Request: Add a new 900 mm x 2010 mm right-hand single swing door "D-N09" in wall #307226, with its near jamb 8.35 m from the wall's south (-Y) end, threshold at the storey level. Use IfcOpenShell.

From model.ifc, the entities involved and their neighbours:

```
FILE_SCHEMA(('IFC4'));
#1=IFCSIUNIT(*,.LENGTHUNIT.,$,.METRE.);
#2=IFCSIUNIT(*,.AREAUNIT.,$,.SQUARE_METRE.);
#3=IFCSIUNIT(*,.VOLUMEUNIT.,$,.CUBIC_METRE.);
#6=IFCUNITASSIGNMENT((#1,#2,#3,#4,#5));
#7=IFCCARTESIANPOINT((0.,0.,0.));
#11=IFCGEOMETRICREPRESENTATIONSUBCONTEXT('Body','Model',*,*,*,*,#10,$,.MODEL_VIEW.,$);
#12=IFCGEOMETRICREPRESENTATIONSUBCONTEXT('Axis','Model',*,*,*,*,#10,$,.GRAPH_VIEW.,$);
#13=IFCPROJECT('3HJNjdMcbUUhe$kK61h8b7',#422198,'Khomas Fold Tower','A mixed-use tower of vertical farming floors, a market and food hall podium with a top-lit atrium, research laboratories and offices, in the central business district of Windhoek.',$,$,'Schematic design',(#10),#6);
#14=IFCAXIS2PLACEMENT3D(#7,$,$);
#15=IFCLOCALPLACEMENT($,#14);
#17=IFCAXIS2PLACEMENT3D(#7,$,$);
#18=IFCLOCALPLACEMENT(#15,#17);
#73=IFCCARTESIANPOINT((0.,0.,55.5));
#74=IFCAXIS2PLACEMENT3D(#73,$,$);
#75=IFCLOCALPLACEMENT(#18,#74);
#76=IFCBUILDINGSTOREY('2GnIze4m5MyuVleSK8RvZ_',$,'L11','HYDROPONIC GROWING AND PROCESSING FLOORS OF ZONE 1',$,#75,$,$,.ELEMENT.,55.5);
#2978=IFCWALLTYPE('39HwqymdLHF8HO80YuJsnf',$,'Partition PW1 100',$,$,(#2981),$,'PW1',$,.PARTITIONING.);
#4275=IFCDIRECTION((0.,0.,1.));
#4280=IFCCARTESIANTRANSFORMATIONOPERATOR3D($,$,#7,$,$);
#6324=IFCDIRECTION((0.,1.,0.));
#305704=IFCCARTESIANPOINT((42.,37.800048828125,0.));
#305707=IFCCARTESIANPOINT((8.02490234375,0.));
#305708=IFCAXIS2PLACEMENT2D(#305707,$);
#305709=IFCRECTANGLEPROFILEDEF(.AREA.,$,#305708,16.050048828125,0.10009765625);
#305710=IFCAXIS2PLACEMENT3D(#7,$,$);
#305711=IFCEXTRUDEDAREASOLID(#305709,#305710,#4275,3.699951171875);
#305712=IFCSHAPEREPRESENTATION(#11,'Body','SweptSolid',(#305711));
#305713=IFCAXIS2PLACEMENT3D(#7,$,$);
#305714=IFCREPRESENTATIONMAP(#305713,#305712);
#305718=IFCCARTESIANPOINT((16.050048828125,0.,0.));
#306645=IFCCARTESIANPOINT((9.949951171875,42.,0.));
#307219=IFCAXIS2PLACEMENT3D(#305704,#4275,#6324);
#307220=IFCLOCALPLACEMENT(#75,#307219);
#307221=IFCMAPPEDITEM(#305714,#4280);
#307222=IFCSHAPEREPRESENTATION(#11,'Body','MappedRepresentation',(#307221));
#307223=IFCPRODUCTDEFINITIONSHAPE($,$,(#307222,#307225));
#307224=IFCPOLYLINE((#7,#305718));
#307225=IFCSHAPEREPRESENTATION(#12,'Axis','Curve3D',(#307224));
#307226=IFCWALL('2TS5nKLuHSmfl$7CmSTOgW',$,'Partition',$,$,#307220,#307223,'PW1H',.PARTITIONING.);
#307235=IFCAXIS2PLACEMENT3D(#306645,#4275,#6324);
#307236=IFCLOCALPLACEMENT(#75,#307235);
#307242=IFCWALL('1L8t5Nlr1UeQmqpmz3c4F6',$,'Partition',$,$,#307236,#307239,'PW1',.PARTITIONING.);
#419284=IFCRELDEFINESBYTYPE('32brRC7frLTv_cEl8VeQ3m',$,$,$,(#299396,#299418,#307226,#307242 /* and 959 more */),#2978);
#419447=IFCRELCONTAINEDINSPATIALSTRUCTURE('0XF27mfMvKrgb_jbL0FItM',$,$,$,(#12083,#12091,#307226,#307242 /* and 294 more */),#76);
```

```python
import numpy as np
import ifcopenshell
import ifcopenshell.api.feature
import ifcopenshell.api.geometry
import ifcopenshell.api.root
import ifcopenshell.api.spatial
import ifcopenshell.geom
import ifcopenshell.util.element
import ifcopenshell.util.placement
import ifcopenshell.util.representation
import ifcopenshell.util.shape
import ifcopenshell.util.unit

model = ifcopenshell.open("model.ifc")
unit_scale = ifcopenshell.util.unit.calculate_unit_scale(model)
settings = ifcopenshell.geom.settings()


def volume(element):
    """Net volume in cubic metres, openings subtracted."""
    shape = ifcopenshell.geom.create_shape(settings, element)
    return ifcopenshell.util.shape.get_volume(shape.geometry)


wall = model.by_guid("2TS5nKLuHSmfl$7CmSTOgW")
storey = ifcopenshell.util.element.get_container(wall, ifc_class="IfcBuildingStorey")
context = ifcopenshell.util.representation.get_context(model, "Model", "Body", "MODEL_VIEW")
before = volume(wall)

width, height, from_end, sill = 0.9, 2.01, 8.35, 0.0  # metres

# The wall runs along its own X axis, and the end named is its -X end.
wall_shape = ifcopenshell.geom.create_shape(settings, wall)
x, y, z = ifcopenshell.util.shape.get_vertices(wall_shape.geometry).T
start = x.min() + from_end
face, thickness = float(y.min()), float(y.max() - y.min())
wall_matrix = ifcopenshell.util.placement.get_local_placement(wall.ObjectPlacement)
level = ifcopenshell.util.placement.get_local_placement(storey.ObjectPlacement)[2, 3]


def in_wall(x, y):
    """Placement at x, y metres in the wall's axes, at sill height."""
    matrix = wall_matrix.copy()
    matrix[:, 3] = wall_matrix @ np.array([x / unit_scale, y / unit_scale, 0.0, 1.0])
    matrix[2, 3] = level + sill / unit_scale
    return matrix


# Opening: a box that overshoots both wall faces by 50 mm.
opening = ifcopenshell.api.root.create_entity(model, ifc_class="IfcOpeningElement", predefined_type="OPENING")
box = ifcopenshell.api.geometry.add_wall_representation(
    model, context=context, length=width, height=height, thickness=thickness + 0.1
)
ifcopenshell.api.geometry.assign_representation(model, product=opening, representation=box)
ifcopenshell.api.geometry.edit_object_placement(model, product=opening, matrix=in_wall(start, face - 0.05), is_si=False)
ifcopenshell.api.feature.add_feature(model, feature=opening, element=wall)

door = ifcopenshell.api.root.create_entity(model, ifc_class="IfcDoor", name="D-N09", predefined_type="DOOR")
door.OverallWidth, door.OverallHeight = width / unit_scale, height / unit_scale
door.OperationType = "SINGLE_SWING_RIGHT"
body = ifcopenshell.api.geometry.add_door_representation(
    model,
    context=context,
    overall_width=door.OverallWidth,
    overall_height=door.OverallHeight,
    operation_type="SINGLE_SWING_RIGHT",
    lining_properties={"LiningDepth": thickness / unit_scale, "ThresholdDepth": thickness / unit_scale},
)
ifcopenshell.api.geometry.assign_representation(model, product=door, representation=body)
ifcopenshell.api.spatial.assign_container(model, products=[door], relating_structure=storey)
ifcopenshell.api.feature.add_filling(model, opening=opening, element=door)

# The lining spans the wall, so the door starts at the wall face.
ifcopenshell.api.geometry.edit_object_placement(model, product=door, matrix=in_wall(start, face), is_si=False)

after = volume(wall)

print(f"wall volume {before:.3f} -> {after:.3f} m3")

model.write("model-out.ifc")
```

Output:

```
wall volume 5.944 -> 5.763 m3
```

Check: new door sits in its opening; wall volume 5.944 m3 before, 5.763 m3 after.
